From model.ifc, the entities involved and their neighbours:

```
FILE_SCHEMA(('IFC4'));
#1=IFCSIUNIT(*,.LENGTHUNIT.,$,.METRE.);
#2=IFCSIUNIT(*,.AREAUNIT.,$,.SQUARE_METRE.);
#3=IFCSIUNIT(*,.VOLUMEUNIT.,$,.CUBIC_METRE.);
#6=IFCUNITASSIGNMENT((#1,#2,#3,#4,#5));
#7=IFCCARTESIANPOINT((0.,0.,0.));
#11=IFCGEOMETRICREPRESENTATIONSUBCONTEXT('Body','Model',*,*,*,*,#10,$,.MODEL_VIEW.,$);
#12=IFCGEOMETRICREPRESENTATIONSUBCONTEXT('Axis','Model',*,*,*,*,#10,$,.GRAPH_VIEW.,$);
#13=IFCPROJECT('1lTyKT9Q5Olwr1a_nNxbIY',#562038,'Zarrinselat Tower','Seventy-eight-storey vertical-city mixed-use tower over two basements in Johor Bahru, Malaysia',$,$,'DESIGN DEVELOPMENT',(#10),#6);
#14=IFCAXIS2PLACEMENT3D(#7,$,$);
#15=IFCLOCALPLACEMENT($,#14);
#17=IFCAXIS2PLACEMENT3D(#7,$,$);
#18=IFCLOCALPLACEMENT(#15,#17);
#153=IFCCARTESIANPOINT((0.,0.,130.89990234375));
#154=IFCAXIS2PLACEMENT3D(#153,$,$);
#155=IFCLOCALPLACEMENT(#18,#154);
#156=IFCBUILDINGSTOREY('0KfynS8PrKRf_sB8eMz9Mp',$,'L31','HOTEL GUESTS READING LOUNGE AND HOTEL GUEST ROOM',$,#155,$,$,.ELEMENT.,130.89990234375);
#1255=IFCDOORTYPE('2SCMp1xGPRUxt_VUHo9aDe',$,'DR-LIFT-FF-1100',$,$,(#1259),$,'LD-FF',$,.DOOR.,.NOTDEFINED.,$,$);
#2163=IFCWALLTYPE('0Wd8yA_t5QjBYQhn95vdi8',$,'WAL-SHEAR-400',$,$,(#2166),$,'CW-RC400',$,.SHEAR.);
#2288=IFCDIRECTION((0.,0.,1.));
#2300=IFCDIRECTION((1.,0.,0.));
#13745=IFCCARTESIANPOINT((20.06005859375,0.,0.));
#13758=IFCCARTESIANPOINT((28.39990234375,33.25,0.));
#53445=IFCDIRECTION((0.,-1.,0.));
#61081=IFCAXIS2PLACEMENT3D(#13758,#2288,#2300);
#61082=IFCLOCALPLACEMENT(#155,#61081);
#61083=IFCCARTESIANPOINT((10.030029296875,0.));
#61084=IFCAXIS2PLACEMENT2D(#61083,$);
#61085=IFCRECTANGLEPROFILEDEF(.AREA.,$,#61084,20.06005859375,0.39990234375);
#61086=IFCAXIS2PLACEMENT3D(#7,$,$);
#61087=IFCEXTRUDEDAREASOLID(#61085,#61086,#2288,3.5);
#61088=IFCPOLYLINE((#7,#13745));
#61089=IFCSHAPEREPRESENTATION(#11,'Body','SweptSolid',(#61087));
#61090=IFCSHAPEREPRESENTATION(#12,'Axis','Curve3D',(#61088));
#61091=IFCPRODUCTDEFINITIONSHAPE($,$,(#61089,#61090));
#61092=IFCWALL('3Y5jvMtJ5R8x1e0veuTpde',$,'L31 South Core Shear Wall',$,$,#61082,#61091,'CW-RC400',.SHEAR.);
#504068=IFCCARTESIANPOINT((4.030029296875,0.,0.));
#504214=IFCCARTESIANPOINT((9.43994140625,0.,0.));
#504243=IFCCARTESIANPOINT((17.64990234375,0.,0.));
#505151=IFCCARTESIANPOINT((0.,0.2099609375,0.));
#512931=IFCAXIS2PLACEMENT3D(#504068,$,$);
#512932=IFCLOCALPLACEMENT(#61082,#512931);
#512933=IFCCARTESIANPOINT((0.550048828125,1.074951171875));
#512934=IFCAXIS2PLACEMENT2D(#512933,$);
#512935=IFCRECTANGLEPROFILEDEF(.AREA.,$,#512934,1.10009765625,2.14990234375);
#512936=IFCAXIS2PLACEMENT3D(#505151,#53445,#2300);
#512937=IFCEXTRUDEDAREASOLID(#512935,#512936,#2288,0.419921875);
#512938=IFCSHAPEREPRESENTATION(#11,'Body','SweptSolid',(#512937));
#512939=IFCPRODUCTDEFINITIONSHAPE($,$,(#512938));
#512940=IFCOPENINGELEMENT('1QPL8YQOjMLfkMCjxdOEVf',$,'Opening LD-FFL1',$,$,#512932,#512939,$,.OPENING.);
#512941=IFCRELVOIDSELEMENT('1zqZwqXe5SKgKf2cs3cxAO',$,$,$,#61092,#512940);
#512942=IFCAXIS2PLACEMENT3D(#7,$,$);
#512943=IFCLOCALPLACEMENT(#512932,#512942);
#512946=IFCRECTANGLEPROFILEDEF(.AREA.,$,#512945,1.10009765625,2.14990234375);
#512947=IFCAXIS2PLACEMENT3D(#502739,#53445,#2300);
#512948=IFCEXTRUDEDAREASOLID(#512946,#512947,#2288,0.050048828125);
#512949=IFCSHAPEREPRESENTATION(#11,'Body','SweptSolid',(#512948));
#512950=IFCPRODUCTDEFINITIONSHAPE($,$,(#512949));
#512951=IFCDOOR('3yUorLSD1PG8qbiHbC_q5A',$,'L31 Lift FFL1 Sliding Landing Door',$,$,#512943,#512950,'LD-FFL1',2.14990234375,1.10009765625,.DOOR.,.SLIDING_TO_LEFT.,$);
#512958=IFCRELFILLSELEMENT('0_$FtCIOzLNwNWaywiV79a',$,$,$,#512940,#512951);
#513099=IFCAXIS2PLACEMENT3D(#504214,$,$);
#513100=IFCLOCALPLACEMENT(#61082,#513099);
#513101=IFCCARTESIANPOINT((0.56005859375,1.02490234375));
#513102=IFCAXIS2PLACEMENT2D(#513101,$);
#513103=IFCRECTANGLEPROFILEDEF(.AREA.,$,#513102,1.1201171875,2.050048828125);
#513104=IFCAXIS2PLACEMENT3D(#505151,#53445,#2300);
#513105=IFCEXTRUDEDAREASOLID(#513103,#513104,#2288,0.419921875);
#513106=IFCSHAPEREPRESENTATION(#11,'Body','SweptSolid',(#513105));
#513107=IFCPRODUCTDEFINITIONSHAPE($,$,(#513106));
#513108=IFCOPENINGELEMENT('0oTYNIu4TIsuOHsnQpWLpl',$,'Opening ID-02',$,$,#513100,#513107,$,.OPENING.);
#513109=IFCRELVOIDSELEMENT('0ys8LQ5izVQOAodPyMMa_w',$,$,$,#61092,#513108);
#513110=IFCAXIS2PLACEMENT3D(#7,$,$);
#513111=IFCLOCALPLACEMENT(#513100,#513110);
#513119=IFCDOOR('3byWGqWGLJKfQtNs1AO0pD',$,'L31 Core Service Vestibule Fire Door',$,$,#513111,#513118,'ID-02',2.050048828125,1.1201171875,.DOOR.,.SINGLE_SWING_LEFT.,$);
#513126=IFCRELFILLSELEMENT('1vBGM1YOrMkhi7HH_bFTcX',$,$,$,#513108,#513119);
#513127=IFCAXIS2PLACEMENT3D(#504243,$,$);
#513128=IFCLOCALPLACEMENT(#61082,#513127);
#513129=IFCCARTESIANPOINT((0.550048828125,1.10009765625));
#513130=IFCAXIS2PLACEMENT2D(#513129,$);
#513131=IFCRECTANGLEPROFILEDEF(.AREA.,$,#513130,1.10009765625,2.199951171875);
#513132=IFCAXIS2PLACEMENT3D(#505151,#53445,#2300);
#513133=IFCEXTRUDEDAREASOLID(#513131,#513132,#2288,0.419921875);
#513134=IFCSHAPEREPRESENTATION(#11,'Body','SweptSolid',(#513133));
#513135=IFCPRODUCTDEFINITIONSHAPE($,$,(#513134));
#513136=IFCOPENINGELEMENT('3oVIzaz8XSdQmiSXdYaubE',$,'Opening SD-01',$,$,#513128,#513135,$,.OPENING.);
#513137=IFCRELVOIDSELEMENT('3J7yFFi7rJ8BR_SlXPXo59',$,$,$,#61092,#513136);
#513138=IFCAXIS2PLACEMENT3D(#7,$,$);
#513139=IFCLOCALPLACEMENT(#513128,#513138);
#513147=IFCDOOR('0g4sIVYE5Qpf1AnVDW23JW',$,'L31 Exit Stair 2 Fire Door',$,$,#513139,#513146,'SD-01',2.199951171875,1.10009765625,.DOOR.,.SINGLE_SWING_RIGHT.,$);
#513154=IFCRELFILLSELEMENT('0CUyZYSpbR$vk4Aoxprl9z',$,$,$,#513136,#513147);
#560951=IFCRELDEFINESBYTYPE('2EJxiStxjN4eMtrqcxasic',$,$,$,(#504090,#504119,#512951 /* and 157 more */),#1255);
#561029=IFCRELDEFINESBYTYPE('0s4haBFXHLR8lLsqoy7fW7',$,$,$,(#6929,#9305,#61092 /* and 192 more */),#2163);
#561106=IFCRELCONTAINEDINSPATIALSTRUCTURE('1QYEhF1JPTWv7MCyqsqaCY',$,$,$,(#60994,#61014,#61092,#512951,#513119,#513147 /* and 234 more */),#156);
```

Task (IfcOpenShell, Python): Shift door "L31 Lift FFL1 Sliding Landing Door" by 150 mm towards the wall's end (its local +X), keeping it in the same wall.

```python
import ifcopenshell
import ifcopenshell.api.geometry
import ifcopenshell.util.placement
import ifcopenshell.util.unit

model = ifcopenshell.open("model.ifc")
unit_scale = ifcopenshell.util.unit.calculate_unit_scale(model)

door = model.by_guid("3yUorLSD1PG8qbiHbC_q5A")
opening = door.FillsVoids[0].RelatingOpeningElement
wall = opening.VoidsElements[0].RelatingBuildingElement

wall_matrix = ifcopenshell.util.placement.get_local_placement(wall.ObjectPlacement)
shift = wall_matrix[:3, 0] * 0.15 / unit_scale
before = ifcopenshell.util.placement.get_local_placement(door.ObjectPlacement)[:3, 3].copy()

# The door is placed relative to its opening, so it follows when the opening moves.
matrix = ifcopenshell.util.placement.get_local_placement(opening.ObjectPlacement)
matrix[:3, 3] += shift
ifcopenshell.api.geometry.edit_object_placement(
    model, product=opening, matrix=matrix, is_si=False, should_transform_children=True
)

after = ifcopenshell.util.placement.get_local_placement(door.ObjectPlacement)[:3, 3]
print("door moved by", (after - before).round(3) + 0.0)

model.write("model_v2.ifc")
```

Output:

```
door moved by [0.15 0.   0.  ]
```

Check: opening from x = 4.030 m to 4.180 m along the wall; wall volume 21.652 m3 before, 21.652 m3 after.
